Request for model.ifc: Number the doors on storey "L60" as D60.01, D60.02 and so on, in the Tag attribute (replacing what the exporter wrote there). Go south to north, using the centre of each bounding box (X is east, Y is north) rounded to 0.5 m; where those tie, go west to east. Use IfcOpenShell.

First a look at what the model holds.

```python
import ifcopenshell
import ifcopenshell.util.element
import ifcopenshell.util.placement

model = ifcopenshell.open("model.ifc")
print(model.schema)
storey = next(s for s in model.by_type("IfcBuildingStorey") if s.Name == "L60")
doors = [e for e in ifcopenshell.util.element.get_decomposition(storey) if e.is_a("IfcDoor")]
for e in sorted(doors, key=lambda e: e.id()):
    origin = ifcopenshell.util.placement.get_local_placement(e.ObjectPlacement)[:3, 3]
    print(e.id(), e.Tag, e.Name, origin.round(2) + 0.0, sep=" | ")
```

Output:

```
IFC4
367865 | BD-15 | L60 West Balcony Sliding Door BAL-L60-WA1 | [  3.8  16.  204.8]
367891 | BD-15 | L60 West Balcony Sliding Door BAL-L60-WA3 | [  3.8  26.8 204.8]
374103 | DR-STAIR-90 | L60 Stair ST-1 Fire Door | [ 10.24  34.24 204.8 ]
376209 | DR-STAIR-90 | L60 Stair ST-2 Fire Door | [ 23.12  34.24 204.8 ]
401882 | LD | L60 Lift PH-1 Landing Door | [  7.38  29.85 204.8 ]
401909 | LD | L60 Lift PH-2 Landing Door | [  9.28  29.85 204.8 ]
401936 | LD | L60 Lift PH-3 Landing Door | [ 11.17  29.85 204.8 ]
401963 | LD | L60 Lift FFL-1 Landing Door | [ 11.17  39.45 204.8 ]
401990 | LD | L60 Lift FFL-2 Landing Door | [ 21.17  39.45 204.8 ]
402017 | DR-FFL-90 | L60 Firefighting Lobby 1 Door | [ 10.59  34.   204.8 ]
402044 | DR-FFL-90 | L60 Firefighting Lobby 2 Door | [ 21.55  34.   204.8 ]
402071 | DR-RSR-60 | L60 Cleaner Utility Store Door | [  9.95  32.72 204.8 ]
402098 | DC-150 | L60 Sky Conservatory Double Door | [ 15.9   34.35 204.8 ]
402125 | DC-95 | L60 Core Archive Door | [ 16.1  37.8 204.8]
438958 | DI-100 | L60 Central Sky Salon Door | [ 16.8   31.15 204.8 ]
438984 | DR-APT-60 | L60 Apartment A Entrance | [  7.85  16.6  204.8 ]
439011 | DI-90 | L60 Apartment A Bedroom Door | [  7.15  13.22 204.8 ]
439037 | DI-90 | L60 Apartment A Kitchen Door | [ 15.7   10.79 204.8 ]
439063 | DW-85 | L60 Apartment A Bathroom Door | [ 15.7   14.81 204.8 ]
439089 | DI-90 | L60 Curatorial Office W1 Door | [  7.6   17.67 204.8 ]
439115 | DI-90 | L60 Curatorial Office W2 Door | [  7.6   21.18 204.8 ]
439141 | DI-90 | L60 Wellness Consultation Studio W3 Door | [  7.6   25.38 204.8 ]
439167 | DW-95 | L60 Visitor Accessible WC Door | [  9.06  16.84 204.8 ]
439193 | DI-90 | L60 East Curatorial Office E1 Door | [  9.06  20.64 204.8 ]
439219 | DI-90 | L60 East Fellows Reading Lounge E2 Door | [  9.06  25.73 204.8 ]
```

```python
import ifcopenshell
import ifcopenshell.geom
import ifcopenshell.util.element
import ifcopenshell.util.shape

model = ifcopenshell.open("model.ifc")
settings = ifcopenshell.geom.settings()
settings.set("use-world-coords", True)


def centre(element):
    shape = ifcopenshell.geom.create_shape(settings, element)
    return ifcopenshell.util.shape.get_bbox_centroid(shape.geometry)


storey = next(s for s in model.by_type("IfcBuildingStorey") if s.Name == "L60")
doors = [e for e in ifcopenshell.util.element.get_decomposition(storey) if e.is_a("IfcDoor")]

# Insertion points can sit at a corner or the storey origin, so sort by the geometry (in metres).
centres = {e: centre(e) for e in doors}
doors.sort(key=lambda e: (round(centres[e][1] / 0.5), centres[e][0]))

for i, e in enumerate(doors, start=1):
    number = f"D60.{i:02d}"
    e.Tag = number
    print(e.id(), number)

model.write("model_rev.ifc")
```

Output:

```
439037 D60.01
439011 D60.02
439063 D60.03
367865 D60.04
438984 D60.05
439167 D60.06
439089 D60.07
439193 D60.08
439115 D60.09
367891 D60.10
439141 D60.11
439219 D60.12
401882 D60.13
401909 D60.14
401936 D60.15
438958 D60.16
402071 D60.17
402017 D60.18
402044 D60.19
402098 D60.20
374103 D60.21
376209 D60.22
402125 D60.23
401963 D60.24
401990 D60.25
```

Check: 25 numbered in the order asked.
